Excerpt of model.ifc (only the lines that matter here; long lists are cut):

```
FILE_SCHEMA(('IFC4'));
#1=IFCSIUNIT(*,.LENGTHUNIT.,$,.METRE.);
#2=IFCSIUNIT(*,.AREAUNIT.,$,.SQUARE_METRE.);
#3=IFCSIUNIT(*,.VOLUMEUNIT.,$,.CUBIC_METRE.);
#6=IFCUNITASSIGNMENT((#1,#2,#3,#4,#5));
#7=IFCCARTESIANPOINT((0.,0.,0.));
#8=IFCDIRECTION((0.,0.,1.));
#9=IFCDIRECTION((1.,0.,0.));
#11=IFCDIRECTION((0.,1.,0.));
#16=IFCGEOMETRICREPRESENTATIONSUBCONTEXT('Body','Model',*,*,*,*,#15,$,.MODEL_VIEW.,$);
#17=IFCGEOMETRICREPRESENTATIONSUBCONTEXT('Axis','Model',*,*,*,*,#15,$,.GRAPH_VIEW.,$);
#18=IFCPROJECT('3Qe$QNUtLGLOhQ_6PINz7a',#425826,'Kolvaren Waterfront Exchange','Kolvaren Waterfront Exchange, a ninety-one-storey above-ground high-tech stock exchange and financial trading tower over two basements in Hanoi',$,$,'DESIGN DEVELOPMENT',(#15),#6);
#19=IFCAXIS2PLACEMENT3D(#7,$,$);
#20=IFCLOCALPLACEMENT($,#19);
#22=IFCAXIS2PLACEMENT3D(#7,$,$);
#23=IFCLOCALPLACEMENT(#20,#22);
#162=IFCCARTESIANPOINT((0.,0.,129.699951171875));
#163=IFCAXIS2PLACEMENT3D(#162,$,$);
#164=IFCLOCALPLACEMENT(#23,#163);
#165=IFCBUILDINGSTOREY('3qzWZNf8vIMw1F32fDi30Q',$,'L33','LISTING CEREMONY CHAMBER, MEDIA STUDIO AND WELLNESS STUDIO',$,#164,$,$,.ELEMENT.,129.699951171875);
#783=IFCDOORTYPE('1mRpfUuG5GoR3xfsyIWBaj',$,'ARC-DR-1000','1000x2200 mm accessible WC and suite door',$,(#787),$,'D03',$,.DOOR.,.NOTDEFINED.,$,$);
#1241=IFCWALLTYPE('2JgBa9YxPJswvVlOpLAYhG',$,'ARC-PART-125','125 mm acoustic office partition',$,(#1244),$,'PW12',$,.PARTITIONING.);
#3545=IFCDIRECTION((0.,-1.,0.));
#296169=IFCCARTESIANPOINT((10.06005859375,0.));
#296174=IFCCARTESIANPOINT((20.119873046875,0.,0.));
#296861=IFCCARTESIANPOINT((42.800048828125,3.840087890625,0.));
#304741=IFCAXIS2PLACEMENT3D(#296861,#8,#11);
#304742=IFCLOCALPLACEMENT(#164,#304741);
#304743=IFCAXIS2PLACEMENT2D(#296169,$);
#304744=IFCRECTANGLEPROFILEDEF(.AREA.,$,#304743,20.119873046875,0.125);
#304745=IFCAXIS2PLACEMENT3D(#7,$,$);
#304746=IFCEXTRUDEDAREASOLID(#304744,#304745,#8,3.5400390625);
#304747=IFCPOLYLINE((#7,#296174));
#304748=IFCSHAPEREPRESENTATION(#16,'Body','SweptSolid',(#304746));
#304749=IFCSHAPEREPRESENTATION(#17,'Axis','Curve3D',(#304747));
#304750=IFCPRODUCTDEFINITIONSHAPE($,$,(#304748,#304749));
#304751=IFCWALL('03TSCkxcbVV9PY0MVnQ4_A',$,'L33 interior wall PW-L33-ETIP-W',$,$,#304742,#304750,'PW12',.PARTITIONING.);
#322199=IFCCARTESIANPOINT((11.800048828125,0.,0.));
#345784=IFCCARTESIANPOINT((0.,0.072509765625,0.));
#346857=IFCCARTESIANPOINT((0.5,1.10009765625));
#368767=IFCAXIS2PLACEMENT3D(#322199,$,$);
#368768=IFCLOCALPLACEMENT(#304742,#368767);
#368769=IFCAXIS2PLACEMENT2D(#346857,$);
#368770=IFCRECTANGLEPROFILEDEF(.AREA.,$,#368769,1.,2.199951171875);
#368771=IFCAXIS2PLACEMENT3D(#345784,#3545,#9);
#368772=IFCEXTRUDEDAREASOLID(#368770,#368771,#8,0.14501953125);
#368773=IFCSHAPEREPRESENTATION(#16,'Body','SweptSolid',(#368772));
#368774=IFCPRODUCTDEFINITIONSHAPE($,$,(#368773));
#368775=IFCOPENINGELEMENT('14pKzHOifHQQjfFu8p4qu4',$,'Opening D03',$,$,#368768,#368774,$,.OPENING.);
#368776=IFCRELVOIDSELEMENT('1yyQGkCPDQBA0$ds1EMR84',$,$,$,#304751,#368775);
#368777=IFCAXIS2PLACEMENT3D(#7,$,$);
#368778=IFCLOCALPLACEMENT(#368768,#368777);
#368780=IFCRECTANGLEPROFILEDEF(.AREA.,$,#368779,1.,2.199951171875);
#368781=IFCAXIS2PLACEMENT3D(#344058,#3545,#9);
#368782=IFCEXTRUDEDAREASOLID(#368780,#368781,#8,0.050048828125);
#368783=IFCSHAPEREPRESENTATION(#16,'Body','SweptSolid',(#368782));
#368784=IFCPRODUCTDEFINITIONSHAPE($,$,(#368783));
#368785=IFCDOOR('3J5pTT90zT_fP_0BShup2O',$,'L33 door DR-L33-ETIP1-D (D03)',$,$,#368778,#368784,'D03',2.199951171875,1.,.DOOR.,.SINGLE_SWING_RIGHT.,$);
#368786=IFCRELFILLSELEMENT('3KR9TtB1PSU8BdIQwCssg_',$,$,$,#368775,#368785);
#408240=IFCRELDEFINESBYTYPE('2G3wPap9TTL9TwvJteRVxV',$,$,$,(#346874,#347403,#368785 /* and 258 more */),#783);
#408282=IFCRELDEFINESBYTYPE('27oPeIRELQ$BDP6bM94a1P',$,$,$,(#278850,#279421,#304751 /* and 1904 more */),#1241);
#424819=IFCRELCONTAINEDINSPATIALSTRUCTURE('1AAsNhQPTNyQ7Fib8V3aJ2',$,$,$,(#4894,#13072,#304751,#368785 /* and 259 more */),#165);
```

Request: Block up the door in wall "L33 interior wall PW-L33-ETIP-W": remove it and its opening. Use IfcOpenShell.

```python
import ifcopenshell
import ifcopenshell.api.feature
import ifcopenshell.api.root
import ifcopenshell.geom
import ifcopenshell.util.shape

model = ifcopenshell.open("model.ifc")
settings = ifcopenshell.geom.settings()


def volume(element):
    """Net volume in cubic metres, openings subtracted."""
    shape = ifcopenshell.geom.create_shape(settings, element)
    return ifcopenshell.util.shape.get_volume(shape.geometry)


door = model.by_guid("3J5pTT90zT_fP_0BShup2O")
opening = door.FillsVoids[0].RelatingOpeningElement
wall = opening.VoidsElements[0].RelatingBuildingElement
before = volume(wall)

ifcopenshell.api.root.remove_product(model, product=door)
ifcopenshell.api.feature.remove_feature(model, feature=opening)

after = volume(wall)

print(f"wall volume {before:.3f} -> {after:.3f} m3")

model.write("model_v2.ifc")
```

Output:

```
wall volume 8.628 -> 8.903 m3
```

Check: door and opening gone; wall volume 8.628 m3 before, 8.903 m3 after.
